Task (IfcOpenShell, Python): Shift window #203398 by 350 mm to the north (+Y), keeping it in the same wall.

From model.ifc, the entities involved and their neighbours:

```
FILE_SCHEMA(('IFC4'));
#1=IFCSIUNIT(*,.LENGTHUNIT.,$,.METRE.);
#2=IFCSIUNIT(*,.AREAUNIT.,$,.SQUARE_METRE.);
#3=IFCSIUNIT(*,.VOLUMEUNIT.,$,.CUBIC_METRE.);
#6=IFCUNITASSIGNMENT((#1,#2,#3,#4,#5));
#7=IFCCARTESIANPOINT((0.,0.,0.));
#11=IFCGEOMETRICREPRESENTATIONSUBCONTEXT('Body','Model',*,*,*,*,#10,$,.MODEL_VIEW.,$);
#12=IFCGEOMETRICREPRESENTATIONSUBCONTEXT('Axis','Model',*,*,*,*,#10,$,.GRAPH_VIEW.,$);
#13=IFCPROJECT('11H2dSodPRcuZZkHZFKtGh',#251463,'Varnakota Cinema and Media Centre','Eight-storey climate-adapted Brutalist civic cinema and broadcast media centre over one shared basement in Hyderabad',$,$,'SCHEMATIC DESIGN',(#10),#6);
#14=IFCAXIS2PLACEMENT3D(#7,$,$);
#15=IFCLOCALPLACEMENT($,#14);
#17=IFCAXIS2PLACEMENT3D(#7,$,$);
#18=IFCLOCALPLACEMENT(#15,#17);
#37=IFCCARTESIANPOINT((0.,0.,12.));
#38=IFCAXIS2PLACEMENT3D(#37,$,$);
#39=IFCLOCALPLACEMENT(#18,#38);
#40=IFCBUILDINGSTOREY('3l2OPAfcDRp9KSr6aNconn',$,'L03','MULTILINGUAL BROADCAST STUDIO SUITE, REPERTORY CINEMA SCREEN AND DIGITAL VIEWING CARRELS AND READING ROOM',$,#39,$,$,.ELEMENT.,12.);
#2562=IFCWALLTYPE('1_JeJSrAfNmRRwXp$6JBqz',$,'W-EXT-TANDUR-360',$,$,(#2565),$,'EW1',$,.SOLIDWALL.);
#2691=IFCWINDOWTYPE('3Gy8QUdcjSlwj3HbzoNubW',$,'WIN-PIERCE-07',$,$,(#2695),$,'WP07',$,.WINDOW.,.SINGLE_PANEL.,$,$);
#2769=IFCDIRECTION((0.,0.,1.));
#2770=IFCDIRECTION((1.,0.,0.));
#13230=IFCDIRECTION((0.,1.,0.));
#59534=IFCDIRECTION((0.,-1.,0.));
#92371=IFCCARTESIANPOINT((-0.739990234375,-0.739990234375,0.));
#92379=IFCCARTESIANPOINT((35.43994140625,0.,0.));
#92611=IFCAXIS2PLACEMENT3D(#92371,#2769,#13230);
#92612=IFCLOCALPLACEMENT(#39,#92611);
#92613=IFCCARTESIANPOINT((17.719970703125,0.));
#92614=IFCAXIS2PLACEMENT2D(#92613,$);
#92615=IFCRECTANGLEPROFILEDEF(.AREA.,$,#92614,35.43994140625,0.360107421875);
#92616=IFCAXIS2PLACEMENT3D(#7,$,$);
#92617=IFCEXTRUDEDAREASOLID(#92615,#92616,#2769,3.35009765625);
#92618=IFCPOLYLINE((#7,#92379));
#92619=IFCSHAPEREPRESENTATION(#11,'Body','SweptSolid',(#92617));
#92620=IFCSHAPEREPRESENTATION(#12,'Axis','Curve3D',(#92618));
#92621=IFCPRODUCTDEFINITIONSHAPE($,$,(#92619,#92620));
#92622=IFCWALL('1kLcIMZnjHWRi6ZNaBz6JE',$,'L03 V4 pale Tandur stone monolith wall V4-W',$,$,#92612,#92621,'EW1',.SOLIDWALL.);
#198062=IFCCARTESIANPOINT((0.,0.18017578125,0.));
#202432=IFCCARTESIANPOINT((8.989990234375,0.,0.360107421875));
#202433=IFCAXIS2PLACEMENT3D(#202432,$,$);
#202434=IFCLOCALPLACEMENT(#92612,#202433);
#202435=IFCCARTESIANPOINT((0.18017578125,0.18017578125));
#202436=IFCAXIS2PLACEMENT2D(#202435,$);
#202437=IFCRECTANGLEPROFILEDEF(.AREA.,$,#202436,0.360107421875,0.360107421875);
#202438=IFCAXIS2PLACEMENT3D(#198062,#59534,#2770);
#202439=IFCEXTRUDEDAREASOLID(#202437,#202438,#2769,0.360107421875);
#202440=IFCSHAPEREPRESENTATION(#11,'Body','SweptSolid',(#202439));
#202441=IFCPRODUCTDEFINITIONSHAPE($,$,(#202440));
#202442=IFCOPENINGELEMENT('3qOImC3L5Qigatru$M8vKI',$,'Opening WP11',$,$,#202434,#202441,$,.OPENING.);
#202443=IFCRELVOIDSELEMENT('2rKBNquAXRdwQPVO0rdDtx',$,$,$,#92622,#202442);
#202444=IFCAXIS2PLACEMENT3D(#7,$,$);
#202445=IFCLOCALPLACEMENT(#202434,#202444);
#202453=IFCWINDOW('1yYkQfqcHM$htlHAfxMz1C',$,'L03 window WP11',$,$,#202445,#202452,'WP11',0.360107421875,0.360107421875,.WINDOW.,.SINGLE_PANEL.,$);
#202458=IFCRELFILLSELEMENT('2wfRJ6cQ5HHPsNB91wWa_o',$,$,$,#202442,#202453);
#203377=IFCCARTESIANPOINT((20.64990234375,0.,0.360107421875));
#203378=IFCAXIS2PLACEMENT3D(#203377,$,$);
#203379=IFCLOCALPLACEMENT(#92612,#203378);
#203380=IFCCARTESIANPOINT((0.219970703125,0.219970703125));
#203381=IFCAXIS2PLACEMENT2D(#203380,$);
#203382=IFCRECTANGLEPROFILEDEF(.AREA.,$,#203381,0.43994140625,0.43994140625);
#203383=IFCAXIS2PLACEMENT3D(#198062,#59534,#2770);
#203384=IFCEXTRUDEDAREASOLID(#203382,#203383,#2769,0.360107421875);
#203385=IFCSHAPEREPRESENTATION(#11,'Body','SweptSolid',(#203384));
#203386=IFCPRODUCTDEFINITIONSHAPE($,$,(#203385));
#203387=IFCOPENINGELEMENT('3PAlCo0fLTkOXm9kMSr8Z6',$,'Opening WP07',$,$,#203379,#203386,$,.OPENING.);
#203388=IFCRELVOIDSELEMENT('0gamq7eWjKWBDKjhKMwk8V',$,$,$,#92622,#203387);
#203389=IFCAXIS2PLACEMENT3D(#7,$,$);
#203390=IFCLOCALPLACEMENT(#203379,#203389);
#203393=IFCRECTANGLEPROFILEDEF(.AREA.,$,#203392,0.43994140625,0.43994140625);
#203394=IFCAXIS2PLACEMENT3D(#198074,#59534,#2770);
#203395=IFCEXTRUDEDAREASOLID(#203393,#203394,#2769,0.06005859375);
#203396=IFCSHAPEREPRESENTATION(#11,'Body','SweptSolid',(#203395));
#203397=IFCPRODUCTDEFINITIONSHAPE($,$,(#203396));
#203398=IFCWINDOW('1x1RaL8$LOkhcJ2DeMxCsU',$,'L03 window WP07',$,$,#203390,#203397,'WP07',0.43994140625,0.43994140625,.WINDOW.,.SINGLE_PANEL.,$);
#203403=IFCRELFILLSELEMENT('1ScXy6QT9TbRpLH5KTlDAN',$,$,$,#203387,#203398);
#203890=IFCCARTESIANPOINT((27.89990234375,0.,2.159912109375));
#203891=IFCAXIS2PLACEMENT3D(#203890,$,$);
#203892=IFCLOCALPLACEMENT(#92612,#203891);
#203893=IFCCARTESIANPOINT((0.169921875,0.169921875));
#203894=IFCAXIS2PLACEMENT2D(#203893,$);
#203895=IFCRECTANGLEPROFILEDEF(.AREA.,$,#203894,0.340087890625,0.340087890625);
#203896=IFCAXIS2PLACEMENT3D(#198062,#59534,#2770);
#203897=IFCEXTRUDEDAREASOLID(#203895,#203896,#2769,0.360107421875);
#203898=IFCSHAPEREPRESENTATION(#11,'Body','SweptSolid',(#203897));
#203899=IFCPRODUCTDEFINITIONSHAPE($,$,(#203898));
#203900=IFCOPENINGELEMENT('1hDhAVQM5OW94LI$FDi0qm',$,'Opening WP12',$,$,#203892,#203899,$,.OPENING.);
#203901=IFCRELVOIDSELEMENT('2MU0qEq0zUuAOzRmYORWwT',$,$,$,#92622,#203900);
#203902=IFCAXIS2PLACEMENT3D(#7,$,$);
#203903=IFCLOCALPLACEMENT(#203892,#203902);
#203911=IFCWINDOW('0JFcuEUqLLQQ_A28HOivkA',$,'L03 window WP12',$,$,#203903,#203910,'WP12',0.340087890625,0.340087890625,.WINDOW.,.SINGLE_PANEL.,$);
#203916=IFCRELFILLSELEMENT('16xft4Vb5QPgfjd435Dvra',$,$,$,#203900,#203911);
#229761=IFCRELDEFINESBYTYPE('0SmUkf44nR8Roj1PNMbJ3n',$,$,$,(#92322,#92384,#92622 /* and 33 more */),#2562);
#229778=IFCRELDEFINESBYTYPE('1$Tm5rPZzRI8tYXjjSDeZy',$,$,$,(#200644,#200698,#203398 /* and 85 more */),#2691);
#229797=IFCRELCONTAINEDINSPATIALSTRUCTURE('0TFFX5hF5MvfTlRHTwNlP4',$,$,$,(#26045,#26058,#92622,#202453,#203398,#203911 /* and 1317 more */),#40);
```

```python
import ifcopenshell
import ifcopenshell.api.geometry
import ifcopenshell.util.placement
import ifcopenshell.util.unit

model = ifcopenshell.open("model.ifc")
unit_scale = ifcopenshell.util.unit.calculate_unit_scale(model)

window = model.by_id(203398)
opening = window.FillsVoids[0].RelatingOpeningElement
wall = opening.VoidsElements[0].RelatingBuildingElement

wall_matrix = ifcopenshell.util.placement.get_local_placement(wall.ObjectPlacement)
shift = wall_matrix[:3, 0] * 0.35 / unit_scale
before = ifcopenshell.util.placement.get_local_placement(window.ObjectPlacement)[:3, 3].copy()

# The window is placed relative to its opening, so it follows when the opening moves.
matrix = ifcopenshell.util.placement.get_local_placement(opening.ObjectPlacement)
matrix[:3, 3] += shift
ifcopenshell.api.geometry.edit_object_placement(
    model, product=opening, matrix=matrix, is_si=False, should_transform_children=True
)

after = ifcopenshell.util.placement.get_local_placement(window.ObjectPlacement)[:3, 3]
print("window moved by", (after - before).round(3) + 0.0)

model.write("model_updated.ifc")
```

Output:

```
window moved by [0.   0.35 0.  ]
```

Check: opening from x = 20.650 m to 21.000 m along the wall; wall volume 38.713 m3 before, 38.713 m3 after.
